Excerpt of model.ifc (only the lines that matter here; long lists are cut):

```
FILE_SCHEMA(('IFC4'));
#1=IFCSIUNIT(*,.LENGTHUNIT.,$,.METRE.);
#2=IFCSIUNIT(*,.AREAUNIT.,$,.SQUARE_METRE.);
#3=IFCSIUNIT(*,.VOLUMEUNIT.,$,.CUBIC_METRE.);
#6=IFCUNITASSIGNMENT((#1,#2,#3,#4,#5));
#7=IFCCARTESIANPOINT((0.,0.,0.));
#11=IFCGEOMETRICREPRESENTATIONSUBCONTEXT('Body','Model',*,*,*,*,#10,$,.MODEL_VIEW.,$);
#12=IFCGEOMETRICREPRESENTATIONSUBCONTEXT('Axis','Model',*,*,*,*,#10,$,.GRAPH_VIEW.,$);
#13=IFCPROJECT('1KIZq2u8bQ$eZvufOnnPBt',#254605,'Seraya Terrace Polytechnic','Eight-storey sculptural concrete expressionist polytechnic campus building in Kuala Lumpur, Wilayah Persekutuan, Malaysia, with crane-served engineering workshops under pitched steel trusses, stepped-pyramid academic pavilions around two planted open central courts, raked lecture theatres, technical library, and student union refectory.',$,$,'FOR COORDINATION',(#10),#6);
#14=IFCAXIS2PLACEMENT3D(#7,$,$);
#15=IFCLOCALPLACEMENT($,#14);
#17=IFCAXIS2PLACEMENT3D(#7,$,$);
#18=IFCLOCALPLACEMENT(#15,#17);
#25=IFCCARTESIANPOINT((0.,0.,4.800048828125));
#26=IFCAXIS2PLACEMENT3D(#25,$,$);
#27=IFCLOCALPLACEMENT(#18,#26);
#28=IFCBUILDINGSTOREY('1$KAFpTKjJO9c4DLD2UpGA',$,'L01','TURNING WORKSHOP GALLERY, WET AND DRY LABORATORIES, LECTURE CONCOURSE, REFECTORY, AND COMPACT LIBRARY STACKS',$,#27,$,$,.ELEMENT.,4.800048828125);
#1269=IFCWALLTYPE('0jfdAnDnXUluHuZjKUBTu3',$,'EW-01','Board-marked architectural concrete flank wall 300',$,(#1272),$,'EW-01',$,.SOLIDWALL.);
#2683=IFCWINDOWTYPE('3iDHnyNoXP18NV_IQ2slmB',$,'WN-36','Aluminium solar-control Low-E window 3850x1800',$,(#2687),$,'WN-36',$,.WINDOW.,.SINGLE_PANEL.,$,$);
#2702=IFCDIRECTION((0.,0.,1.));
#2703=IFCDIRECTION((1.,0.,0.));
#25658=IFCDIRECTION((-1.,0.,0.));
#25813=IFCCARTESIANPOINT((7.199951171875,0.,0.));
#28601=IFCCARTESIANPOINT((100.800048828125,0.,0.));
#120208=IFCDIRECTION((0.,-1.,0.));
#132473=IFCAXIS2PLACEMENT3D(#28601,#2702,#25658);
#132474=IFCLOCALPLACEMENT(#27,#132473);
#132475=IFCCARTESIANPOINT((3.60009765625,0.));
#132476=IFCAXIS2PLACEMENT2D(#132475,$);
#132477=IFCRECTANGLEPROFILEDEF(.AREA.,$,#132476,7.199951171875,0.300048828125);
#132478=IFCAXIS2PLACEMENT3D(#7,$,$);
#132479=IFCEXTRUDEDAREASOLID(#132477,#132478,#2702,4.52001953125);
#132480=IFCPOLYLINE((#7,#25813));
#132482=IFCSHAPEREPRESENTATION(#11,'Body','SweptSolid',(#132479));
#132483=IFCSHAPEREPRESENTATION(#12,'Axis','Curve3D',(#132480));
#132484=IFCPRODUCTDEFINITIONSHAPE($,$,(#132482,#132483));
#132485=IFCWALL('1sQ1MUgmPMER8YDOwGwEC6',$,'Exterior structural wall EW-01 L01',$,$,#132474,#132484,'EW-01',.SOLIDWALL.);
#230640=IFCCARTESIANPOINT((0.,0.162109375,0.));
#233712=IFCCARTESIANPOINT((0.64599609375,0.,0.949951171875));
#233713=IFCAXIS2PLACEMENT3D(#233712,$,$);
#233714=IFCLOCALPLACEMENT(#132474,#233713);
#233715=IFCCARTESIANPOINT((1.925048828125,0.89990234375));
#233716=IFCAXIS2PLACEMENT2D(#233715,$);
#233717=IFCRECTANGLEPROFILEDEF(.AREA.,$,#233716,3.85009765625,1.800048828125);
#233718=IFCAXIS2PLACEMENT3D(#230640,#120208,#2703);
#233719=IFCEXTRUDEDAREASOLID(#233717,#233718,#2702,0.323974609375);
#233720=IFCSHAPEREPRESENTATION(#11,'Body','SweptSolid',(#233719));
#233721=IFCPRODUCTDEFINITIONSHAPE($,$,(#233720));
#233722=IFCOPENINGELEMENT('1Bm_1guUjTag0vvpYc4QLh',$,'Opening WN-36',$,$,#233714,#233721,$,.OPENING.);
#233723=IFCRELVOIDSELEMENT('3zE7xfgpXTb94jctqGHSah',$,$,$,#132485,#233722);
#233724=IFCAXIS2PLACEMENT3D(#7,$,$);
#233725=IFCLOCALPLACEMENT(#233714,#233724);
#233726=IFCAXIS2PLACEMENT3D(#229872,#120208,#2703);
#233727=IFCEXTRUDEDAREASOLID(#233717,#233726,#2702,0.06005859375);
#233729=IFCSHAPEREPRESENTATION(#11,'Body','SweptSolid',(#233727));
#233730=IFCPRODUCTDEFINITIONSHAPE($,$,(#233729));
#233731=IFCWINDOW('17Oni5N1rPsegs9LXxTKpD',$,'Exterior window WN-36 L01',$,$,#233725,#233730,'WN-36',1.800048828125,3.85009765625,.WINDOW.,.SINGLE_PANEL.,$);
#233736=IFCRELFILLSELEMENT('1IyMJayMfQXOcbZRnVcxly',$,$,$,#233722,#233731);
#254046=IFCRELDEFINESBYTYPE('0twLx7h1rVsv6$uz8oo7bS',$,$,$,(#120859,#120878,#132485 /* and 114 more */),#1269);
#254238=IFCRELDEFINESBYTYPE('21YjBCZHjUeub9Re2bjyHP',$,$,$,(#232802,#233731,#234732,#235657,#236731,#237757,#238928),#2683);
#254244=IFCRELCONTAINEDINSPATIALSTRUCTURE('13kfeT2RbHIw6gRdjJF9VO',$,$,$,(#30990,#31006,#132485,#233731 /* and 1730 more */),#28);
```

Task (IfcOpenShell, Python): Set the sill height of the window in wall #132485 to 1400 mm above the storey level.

```python
import numpy as np
import ifcopenshell
import ifcopenshell.api.geometry
import ifcopenshell.geom
import ifcopenshell.util.element
import ifcopenshell.util.placement
import ifcopenshell.util.shape
import ifcopenshell.util.unit

model = ifcopenshell.open("model.ifc")
unit_scale = ifcopenshell.util.unit.calculate_unit_scale(model)

window = model.by_guid("17Oni5N1rPsegs9LXxTKpD")
opening = window.FillsVoids[0].RelatingOpeningElement
storey = ifcopenshell.util.element.get_container(window, ifc_class="IfcBuildingStorey")
level = ifcopenshell.util.placement.get_local_placement(storey.ObjectPlacement)[2, 3]

# The opening's origin need not be at the sill, so measure its lowest point.
shape = ifcopenshell.geom.create_shape(ifcopenshell.geom.settings(), opening)
bottom = ifcopenshell.util.shape.get_shape_bottom_elevation(shape, shape.geometry) / unit_scale
dz = level + 1.4 / unit_scale - bottom

shift = np.array([0.0, 0.0, dz])
# The window is placed relative to its opening, so it follows when the opening moves.
matrix = ifcopenshell.util.placement.get_local_placement(opening.ObjectPlacement)
matrix[:3, 3] += shift
ifcopenshell.api.geometry.edit_object_placement(
    model, product=opening, matrix=matrix, is_si=False, should_transform_children=True
)

print(f"moved by {dz * unit_scale:+.3f} m")

model.write("model_updated.ifc")
```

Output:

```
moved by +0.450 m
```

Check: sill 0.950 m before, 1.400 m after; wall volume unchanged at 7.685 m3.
